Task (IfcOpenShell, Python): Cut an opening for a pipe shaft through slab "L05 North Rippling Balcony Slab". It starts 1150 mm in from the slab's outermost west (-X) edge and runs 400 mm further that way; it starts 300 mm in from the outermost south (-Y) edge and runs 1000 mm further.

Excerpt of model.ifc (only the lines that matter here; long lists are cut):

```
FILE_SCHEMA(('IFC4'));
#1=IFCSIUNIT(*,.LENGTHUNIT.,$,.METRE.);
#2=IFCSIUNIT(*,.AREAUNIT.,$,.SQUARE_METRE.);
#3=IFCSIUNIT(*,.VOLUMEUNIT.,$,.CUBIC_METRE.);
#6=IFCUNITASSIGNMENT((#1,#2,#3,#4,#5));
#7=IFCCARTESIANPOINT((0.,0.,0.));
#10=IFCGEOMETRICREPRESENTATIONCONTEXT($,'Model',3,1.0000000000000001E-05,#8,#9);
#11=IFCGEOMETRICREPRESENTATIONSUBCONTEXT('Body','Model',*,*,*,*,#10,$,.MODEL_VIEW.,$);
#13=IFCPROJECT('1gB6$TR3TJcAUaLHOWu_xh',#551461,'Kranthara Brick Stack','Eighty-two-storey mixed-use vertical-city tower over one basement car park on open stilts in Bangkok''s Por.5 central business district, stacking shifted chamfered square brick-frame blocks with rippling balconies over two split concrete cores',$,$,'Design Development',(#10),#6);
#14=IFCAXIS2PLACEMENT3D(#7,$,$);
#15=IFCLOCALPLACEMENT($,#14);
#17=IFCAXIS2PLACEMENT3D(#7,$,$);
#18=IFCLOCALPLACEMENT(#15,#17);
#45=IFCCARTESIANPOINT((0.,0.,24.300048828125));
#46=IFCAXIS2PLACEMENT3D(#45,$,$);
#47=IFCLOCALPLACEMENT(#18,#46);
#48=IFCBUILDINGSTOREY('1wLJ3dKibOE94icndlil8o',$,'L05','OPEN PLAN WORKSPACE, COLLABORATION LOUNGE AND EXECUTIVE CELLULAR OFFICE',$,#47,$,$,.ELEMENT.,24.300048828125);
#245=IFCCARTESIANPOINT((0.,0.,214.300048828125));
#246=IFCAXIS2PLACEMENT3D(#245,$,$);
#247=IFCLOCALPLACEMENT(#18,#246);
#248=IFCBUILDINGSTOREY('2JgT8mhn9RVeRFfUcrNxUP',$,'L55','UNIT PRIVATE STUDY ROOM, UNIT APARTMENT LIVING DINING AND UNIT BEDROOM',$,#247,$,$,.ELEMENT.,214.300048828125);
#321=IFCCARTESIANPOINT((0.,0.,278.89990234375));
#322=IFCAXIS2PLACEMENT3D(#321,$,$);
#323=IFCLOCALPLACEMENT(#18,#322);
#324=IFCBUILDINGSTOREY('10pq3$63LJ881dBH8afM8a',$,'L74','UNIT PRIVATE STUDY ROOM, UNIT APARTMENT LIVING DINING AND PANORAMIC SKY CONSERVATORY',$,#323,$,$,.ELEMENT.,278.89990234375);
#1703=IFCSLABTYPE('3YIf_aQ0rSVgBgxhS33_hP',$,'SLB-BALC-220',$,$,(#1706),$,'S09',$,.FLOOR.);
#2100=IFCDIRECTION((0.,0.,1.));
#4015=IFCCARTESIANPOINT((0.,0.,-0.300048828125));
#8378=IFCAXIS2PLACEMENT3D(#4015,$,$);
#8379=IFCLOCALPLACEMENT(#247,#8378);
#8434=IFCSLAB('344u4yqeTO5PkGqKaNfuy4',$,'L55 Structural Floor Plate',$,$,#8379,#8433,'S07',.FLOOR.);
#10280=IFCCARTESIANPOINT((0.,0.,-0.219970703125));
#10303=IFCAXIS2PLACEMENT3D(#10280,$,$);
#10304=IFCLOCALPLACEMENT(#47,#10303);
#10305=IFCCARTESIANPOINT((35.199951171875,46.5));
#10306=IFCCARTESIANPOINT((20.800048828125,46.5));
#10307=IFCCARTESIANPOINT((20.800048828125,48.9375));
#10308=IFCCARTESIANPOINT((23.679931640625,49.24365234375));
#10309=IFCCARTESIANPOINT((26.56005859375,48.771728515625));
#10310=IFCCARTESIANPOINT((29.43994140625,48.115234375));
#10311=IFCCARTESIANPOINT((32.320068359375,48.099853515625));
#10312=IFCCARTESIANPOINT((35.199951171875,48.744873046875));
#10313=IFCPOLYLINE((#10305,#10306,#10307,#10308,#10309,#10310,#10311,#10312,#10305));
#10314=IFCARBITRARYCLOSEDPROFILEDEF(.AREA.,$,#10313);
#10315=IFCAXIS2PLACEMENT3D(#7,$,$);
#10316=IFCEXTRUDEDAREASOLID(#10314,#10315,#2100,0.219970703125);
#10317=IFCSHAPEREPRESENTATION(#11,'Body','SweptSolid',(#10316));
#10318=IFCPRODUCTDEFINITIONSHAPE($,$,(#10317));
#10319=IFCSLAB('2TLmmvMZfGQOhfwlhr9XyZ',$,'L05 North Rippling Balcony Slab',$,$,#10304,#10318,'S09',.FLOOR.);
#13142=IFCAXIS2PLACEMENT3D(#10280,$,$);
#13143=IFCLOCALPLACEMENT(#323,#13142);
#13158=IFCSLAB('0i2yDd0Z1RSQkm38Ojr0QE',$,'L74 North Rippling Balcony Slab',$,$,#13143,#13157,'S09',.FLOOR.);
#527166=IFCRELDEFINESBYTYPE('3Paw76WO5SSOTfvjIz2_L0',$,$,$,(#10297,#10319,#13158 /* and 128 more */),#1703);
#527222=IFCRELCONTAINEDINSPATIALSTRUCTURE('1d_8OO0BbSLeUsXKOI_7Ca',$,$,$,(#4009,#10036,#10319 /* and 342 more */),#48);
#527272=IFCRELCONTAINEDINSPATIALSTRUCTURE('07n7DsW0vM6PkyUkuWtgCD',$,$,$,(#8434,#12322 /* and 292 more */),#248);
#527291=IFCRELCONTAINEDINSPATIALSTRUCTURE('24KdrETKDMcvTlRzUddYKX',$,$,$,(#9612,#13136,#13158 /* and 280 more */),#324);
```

```python
import numpy as np
import ifcopenshell
import ifcopenshell.api.feature
import ifcopenshell.api.geometry
import ifcopenshell.api.root
import ifcopenshell.geom
import ifcopenshell.util.placement
import ifcopenshell.util.representation
import ifcopenshell.util.shape
import ifcopenshell.util.unit

model = ifcopenshell.open("model.ifc")
unit_scale = ifcopenshell.util.unit.calculate_unit_scale(model)
settings = ifcopenshell.geom.settings()


def volume(element):
    """Net volume in cubic metres, openings subtracted."""
    shape = ifcopenshell.geom.create_shape(settings, element)
    return ifcopenshell.util.shape.get_volume(shape.geometry)


slab = model.by_id(10319)
before = volume(slab)

# Extent in the slab's own axes, in metres. The edges named are its -X and -Y sides.
slab_shape = ifcopenshell.geom.create_shape(settings, slab)
vertices = ifcopenshell.util.shape.get_vertices(slab_shape.geometry)
x_min, y_min, bottom = vertices.min(axis=0)
top = vertices[:, 2].max()

opening = ifcopenshell.api.root.create_entity(model, ifc_class="IfcOpeningElement", name="Pipe shaft opening", predefined_type="OPENING")
context = ifcopenshell.util.representation.get_context(model, "Model", "Body", "MODEL_VIEW")
width, depth = 0.4, 1
outline = [(0.0, 0.0), (width, 0.0), (width, depth), (0.0, depth), (0.0, 0.0)]
# Overshoot both faces by 50 mm so the cut is clean.
shape = ifcopenshell.api.geometry.add_slab_representation(
    model, context=context, depth=top - bottom + 0.1, polyline=outline
)
ifcopenshell.api.geometry.assign_representation(model, product=opening, representation=shape)

matrix = ifcopenshell.util.placement.get_local_placement(slab.ObjectPlacement)
matrix[:, 3] = matrix @ np.append(np.array([x_min + 1.15, y_min + 0.3, bottom - 0.05]) / unit_scale, 1.0)
ifcopenshell.api.geometry.edit_object_placement(model, product=opening, matrix=matrix, is_si=False)
ifcopenshell.api.feature.add_feature(model, feature=opening, element=slab)

after = volume(slab)

print(f"slab volume {before:.3f} -> {after:.3f} m3")

model.write("model_edited.ifc")
```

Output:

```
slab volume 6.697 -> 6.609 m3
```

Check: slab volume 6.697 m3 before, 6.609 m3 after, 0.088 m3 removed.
